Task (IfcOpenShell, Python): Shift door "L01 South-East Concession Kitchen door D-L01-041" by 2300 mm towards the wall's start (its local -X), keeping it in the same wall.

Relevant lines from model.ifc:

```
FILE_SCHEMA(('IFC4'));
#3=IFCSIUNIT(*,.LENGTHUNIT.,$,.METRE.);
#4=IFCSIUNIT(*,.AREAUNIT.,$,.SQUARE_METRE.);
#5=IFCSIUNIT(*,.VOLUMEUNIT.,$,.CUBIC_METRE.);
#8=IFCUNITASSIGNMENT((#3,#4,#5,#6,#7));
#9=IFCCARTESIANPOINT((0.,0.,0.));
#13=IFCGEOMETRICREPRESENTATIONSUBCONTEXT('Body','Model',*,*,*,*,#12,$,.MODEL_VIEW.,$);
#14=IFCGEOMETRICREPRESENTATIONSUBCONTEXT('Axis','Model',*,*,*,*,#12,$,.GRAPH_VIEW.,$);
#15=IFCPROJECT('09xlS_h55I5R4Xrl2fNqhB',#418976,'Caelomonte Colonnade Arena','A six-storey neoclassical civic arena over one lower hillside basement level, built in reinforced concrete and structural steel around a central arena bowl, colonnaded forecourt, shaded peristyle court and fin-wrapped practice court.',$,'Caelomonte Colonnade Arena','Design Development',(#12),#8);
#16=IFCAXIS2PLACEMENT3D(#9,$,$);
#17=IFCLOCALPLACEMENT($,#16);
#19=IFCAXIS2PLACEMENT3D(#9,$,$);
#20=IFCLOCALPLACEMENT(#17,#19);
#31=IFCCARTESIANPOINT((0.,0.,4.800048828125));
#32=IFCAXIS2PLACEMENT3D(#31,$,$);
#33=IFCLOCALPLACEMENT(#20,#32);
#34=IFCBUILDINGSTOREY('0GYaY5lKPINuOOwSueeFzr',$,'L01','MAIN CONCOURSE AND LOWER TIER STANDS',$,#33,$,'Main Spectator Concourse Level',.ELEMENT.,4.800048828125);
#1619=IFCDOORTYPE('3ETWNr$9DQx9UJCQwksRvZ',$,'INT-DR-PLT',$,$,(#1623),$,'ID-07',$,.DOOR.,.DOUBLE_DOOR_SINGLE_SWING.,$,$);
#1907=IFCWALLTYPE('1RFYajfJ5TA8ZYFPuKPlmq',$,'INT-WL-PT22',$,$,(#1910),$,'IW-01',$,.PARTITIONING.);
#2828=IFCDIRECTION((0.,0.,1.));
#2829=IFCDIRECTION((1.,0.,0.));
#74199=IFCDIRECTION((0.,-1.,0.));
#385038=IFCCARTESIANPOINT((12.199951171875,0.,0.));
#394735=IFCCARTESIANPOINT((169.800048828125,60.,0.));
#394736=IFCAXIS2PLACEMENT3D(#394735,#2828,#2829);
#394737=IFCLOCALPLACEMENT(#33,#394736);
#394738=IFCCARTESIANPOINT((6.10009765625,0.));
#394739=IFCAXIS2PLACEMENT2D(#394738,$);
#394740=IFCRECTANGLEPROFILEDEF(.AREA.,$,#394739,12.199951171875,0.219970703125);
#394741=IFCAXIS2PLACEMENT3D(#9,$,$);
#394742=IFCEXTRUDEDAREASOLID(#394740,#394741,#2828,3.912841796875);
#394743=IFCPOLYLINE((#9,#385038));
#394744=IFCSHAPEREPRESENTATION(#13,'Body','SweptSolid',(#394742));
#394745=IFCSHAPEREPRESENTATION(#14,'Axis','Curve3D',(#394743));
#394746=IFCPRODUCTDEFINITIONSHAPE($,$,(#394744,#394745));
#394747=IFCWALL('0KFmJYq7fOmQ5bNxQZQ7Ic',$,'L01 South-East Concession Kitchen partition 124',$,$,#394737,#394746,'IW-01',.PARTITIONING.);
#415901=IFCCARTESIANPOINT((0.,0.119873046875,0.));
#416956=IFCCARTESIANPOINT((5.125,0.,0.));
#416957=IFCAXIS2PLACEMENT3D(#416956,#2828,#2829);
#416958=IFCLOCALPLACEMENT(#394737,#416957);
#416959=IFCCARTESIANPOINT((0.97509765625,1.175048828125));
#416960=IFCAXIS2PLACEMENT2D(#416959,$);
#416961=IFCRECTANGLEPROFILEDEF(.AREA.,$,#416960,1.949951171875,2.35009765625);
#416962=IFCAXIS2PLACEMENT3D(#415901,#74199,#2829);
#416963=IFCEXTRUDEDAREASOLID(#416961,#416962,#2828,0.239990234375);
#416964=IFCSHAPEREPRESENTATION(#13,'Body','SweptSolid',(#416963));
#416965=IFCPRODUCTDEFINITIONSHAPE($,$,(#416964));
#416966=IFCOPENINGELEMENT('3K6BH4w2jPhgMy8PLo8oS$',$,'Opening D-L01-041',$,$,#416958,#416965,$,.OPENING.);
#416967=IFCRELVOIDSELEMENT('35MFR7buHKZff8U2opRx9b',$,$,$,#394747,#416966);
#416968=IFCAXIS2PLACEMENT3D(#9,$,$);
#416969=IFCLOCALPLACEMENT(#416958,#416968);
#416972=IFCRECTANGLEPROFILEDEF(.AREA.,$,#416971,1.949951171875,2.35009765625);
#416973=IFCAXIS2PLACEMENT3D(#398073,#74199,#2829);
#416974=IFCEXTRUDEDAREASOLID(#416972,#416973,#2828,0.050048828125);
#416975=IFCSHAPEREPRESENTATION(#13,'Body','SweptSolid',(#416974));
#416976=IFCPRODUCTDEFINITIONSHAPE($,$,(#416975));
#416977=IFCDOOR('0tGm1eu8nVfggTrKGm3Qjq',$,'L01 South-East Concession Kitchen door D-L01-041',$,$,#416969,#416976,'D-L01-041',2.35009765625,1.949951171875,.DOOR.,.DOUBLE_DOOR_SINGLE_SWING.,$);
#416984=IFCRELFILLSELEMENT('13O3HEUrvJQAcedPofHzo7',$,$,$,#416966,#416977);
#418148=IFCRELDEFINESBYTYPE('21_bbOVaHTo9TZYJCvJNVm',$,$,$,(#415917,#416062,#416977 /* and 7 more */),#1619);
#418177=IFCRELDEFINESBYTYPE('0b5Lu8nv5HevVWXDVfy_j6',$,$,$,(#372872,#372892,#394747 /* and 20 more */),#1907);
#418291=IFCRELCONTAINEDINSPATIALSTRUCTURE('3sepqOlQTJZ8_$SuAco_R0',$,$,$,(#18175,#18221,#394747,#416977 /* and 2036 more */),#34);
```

```python
import ifcopenshell
import ifcopenshell.api.geometry
import ifcopenshell.util.placement
import ifcopenshell.util.unit

model = ifcopenshell.open("model.ifc")
unit_scale = ifcopenshell.util.unit.calculate_unit_scale(model)

door = model.by_guid("0tGm1eu8nVfggTrKGm3Qjq")
opening = door.FillsVoids[0].RelatingOpeningElement
wall = opening.VoidsElements[0].RelatingBuildingElement

wall_matrix = ifcopenshell.util.placement.get_local_placement(wall.ObjectPlacement)
shift = wall_matrix[:3, 0] * -2.3 / unit_scale
before = ifcopenshell.util.placement.get_local_placement(door.ObjectPlacement)[:3, 3].copy()

# The door is placed relative to its opening, so it follows when the opening moves.
matrix = ifcopenshell.util.placement.get_local_placement(opening.ObjectPlacement)
matrix[:3, 3] += shift
ifcopenshell.api.geometry.edit_object_placement(
    model, product=opening, matrix=matrix, is_si=False, should_transform_children=True
)

after = ifcopenshell.util.placement.get_local_placement(door.ObjectPlacement)[:3, 3]
print("door moved by", (after - before).round(3) + 0.0)

model.write("model_rev.ifc")
```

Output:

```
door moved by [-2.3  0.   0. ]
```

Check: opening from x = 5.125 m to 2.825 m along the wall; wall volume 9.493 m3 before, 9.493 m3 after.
